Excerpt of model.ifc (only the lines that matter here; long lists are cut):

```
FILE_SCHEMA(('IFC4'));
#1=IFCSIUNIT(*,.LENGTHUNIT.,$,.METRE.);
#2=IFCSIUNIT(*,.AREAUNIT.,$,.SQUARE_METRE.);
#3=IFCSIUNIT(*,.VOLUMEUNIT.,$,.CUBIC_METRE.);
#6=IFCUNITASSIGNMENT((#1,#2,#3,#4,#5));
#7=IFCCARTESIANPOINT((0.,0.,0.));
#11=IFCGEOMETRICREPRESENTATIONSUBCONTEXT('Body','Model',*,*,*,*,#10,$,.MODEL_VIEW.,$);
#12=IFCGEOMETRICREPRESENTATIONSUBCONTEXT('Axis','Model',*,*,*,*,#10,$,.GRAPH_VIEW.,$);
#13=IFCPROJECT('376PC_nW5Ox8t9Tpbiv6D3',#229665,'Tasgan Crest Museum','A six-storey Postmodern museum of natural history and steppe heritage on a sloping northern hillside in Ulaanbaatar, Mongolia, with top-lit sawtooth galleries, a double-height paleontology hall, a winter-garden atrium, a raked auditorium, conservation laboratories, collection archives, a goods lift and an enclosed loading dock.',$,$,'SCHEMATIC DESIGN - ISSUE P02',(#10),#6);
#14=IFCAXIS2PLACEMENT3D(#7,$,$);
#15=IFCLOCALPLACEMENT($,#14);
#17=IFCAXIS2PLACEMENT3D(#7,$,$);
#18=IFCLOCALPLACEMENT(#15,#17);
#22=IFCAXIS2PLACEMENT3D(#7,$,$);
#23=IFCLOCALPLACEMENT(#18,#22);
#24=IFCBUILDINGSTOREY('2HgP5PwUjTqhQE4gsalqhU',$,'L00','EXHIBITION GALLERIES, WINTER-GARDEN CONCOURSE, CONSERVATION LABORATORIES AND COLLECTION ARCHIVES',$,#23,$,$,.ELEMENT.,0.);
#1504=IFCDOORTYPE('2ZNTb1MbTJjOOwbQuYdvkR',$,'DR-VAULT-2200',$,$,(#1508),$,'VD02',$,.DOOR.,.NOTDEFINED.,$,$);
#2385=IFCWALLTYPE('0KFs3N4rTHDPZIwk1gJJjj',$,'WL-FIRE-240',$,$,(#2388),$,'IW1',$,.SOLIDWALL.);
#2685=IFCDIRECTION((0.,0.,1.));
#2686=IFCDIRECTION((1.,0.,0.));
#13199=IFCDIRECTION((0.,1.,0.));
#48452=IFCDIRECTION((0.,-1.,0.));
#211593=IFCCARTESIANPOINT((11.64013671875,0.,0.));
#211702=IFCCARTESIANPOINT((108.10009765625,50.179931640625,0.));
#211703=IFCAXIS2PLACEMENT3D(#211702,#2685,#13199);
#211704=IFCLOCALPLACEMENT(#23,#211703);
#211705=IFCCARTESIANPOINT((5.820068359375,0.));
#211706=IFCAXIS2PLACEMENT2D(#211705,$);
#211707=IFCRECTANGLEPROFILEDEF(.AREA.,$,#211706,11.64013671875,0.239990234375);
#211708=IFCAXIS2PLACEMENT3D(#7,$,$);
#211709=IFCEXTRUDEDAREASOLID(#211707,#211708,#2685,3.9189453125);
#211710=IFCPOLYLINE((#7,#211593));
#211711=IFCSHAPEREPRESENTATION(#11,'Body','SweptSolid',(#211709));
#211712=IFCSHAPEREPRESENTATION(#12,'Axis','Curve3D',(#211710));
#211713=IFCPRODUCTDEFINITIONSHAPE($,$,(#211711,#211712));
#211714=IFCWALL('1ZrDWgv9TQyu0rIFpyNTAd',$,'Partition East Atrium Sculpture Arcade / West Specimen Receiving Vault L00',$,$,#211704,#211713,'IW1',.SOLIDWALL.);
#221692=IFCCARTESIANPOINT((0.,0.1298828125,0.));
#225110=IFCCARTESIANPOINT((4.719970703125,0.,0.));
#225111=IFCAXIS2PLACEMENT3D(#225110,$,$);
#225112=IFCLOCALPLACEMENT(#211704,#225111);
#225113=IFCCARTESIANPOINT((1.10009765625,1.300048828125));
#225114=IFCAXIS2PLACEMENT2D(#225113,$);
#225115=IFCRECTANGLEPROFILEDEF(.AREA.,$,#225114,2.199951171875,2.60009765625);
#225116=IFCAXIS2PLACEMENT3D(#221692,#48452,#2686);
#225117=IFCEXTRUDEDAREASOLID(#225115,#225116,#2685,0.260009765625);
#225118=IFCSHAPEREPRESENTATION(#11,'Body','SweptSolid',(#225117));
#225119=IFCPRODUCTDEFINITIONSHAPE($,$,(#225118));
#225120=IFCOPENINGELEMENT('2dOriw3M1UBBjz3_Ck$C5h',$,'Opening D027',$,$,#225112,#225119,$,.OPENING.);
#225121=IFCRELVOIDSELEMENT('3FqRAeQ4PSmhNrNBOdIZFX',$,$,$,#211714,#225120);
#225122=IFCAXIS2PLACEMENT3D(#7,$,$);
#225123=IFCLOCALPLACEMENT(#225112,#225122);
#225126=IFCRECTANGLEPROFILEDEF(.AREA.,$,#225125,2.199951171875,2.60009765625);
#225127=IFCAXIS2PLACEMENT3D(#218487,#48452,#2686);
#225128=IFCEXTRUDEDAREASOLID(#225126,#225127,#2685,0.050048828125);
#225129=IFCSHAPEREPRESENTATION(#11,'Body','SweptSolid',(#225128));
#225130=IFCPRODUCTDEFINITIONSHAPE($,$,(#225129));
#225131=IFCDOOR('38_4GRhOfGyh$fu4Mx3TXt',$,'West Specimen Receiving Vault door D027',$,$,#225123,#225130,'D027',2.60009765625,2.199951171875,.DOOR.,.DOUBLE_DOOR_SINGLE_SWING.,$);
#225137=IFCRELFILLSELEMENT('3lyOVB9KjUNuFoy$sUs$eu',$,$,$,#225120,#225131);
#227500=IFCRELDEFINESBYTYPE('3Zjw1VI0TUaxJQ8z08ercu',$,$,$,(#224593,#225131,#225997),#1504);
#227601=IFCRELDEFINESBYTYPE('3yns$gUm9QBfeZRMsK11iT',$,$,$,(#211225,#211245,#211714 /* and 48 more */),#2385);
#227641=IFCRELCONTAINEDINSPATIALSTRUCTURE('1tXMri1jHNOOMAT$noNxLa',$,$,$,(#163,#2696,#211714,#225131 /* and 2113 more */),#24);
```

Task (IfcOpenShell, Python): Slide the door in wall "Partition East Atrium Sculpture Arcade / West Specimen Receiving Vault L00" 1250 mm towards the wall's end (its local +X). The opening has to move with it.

```python
import ifcopenshell
import ifcopenshell.api.geometry
import ifcopenshell.util.placement

model = ifcopenshell.open("model.ifc")

door = model.by_guid("38_4GRhOfGyh$fu4Mx3TXt")
opening = door.FillsVoids[0].RelatingOpeningElement
wall = opening.VoidsElements[0].RelatingBuildingElement

wall_matrix = ifcopenshell.util.placement.get_local_placement(wall.ObjectPlacement)
shift = wall_matrix[:3, 0] * 1.25
before = ifcopenshell.util.placement.get_local_placement(door.ObjectPlacement)[:3, 3].copy()

# The door is placed relative to its opening, so it follows when the opening moves.
matrix = ifcopenshell.util.placement.get_local_placement(opening.ObjectPlacement)
matrix[:3, 3] += shift
ifcopenshell.api.geometry.edit_object_placement(
    model, product=opening, matrix=matrix, is_si=False, should_transform_children=True
)

after = ifcopenshell.util.placement.get_local_placement(door.ObjectPlacement)[:3, 3]
print("door moved by", (after - before).round(3) + 0.0)

model.write("model_v2.ifc")
```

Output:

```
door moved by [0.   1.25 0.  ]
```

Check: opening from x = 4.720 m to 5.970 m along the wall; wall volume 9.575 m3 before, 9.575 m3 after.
